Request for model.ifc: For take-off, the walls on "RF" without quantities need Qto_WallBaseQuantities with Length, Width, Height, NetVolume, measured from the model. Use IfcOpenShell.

First a look at what the model holds.

```python
import ifcopenshell
import ifcopenshell.util.element
import ifcopenshell.util.unit

model = ifcopenshell.open("model.ifc")
print(model.schema)
for unit_type in ("LENGTHUNIT", "AREAUNIT", "VOLUMEUNIT"):
    print(unit_type, ifcopenshell.util.unit.calculate_unit_scale(model, unit_type))
storey = next(s for s in model.by_type("IfcBuildingStorey") if s.Name == "RF")
walls = [e for e in ifcopenshell.util.element.get_decomposition(storey) if e.is_a("IfcWall")]
for e in sorted(walls, key=lambda e: e.id()):
    print(e.id(), e.is_a(), e.Name, list(ifcopenshell.util.element.get_psets(e, qtos_only=True)), sep=" | ")
```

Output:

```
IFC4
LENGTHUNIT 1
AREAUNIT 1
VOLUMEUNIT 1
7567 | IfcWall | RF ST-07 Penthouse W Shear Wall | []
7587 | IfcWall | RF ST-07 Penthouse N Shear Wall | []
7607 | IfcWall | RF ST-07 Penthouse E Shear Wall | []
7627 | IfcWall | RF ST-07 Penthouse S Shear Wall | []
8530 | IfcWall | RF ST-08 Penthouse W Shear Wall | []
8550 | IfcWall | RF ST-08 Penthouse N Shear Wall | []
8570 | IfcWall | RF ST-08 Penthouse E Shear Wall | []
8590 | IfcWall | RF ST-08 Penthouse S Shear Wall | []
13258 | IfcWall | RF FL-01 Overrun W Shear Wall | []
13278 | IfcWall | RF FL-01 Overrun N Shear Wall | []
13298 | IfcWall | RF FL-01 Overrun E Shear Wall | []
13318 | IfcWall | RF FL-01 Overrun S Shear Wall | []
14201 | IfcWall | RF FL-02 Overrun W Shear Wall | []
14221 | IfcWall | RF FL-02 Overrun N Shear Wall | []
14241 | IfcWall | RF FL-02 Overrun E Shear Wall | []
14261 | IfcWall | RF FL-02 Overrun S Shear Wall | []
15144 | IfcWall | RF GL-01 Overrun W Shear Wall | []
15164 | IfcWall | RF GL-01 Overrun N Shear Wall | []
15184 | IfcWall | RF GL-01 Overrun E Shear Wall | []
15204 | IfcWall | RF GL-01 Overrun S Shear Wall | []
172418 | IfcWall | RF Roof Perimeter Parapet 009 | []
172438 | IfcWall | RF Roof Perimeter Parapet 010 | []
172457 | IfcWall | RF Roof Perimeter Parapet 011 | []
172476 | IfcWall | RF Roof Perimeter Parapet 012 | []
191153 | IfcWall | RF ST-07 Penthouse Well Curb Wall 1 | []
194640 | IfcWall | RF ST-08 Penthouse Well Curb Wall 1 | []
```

```python
import ifcopenshell
import ifcopenshell.api.pset
import ifcopenshell.geom
import ifcopenshell.util.element
import ifcopenshell.util.shape
import ifcopenshell.util.unit

model = ifcopenshell.open("model.ifc")
unit_scale = ifcopenshell.util.unit.calculate_unit_scale(model)
volume_scale = ifcopenshell.util.unit.calculate_unit_scale(model, "VOLUMEUNIT")
settings = ifcopenshell.geom.settings()

storey = next(s for s in model.by_type("IfcBuildingStorey") if s.Name == "RF")
walls = [e for e in ifcopenshell.util.element.get_decomposition(storey) if e.is_a("IfcWall")]

for e in sorted(walls, key=lambda e: e.id()):
    if ifcopenshell.util.element.get_psets(e, qtos_only=True, should_inherit=False):
        continue
    # Geometry comes back in metres, in the element's own axes.
    shape = ifcopenshell.geom.create_shape(settings, e)
    values = {
        "Length": ifcopenshell.util.shape.get_x(shape.geometry) / unit_scale,
        "Width": ifcopenshell.util.shape.get_y(shape.geometry) / unit_scale,
        "Height": ifcopenshell.util.shape.get_z(shape.geometry) / unit_scale,
        "NetVolume": ifcopenshell.util.shape.get_volume(shape.geometry) / volume_scale,
    }
    qto = ifcopenshell.api.pset.add_qto(model, product=e, name="Qto_WallBaseQuantities")
    ifcopenshell.api.pset.edit_qto(model, qto=qto, properties=values)
    print(e.id(), {k: round(v, 3) for k, v in values.items()})

model.write("model_edited.ifc")
```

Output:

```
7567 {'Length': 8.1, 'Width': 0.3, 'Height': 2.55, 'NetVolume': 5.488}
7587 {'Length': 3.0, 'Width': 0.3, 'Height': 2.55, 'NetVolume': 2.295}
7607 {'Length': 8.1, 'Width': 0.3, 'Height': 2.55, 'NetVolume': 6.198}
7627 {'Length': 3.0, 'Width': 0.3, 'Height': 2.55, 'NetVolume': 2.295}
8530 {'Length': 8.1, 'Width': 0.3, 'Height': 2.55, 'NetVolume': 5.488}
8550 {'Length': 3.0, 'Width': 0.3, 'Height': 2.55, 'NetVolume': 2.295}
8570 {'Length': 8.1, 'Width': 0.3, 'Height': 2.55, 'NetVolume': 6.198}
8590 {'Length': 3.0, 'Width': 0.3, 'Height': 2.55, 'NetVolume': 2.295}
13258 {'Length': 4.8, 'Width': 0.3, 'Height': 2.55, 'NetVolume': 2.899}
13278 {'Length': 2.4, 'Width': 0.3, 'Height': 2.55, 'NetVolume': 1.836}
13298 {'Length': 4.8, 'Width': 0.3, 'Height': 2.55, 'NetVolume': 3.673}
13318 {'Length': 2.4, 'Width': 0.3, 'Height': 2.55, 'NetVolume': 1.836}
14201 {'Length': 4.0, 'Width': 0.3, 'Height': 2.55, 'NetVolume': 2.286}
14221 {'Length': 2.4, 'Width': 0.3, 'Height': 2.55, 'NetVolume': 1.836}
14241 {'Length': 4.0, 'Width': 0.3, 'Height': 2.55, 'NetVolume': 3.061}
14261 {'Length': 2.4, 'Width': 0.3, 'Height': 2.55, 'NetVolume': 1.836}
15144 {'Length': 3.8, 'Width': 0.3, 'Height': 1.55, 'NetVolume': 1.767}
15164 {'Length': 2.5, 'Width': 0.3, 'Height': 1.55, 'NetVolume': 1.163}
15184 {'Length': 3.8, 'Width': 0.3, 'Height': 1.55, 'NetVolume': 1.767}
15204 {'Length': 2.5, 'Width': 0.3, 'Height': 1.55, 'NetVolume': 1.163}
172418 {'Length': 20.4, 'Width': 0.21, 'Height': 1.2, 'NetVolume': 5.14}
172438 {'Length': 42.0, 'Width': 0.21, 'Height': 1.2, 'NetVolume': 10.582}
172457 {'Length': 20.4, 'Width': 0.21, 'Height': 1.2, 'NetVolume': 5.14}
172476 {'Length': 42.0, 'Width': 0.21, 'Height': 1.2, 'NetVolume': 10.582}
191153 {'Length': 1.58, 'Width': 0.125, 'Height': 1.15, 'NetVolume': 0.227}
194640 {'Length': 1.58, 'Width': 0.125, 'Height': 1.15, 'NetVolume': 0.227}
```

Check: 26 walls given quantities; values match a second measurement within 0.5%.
